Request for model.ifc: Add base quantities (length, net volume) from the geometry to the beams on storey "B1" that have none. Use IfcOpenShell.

First a look at what the model holds.

```python
import ifcopenshell
import ifcopenshell.util.element
import ifcopenshell.util.unit

model = ifcopenshell.open("model.ifc")
print(model.schema)
for unit_type in ("LENGTHUNIT", "AREAUNIT", "VOLUMEUNIT"):
    print(unit_type, ifcopenshell.util.unit.calculate_unit_scale(model, unit_type))
storey = next(s for s in model.by_type("IfcBuildingStorey") if s.Name == "B1")
beams = [e for e in ifcopenshell.util.element.get_decomposition(storey) if e.is_a("IfcBeam")]
for e in sorted(beams, key=lambda e: e.id()):
    print(e.id(), e.is_a(), e.Name, list(ifcopenshell.util.element.get_psets(e, qtos_only=True)), sep=" | ")
```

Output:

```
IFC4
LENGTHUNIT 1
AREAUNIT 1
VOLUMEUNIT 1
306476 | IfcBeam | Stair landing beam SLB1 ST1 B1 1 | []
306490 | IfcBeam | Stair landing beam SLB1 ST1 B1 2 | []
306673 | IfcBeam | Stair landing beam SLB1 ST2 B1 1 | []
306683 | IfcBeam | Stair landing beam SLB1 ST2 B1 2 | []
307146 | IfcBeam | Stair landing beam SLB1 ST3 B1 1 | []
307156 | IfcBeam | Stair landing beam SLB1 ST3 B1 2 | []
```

```python
import ifcopenshell
import ifcopenshell.api.pset
import ifcopenshell.geom
import ifcopenshell.util.element
import ifcopenshell.util.shape
import ifcopenshell.util.unit

model = ifcopenshell.open("model.ifc")
unit_scale = ifcopenshell.util.unit.calculate_unit_scale(model)
volume_scale = ifcopenshell.util.unit.calculate_unit_scale(model, "VOLUMEUNIT")
settings = ifcopenshell.geom.settings()

storey = next(s for s in model.by_type("IfcBuildingStorey") if s.Name == "B1")
beams = [e for e in ifcopenshell.util.element.get_decomposition(storey) if e.is_a("IfcBeam")]

for e in sorted(beams, key=lambda e: e.id()):
    if ifcopenshell.util.element.get_psets(e, qtos_only=True, should_inherit=False):
        continue
    # Geometry comes back in metres, in the element's own axes.
    shape = ifcopenshell.geom.create_shape(settings, e)
    values = {
        "Length": ifcopenshell.util.shape.get_max_xyz(shape.geometry) / unit_scale,
        "NetVolume": ifcopenshell.util.shape.get_volume(shape.geometry) / volume_scale,
    }
    qto = ifcopenshell.api.pset.add_qto(model, product=e, name="Qto_BeamBaseQuantities")
    ifcopenshell.api.pset.edit_qto(model, qto=qto, properties=values)
    print(e.id(), {k: round(v, 3) for k, v in values.items()})

model.write("model_edited.ifc")
```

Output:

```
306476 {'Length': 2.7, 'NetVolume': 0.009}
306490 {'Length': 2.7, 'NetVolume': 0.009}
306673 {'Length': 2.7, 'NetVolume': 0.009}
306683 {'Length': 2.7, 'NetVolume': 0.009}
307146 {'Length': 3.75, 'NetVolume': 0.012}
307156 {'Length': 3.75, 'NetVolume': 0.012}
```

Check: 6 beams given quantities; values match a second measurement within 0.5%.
